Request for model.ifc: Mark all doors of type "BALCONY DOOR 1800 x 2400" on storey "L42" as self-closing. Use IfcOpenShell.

First a look at what the model holds.

```python
import ifcopenshell
import ifcopenshell.util.element

model = ifcopenshell.open("model.ifc")
print(model.schema)
storey = next(s for s in model.by_type("IfcBuildingStorey") if s.Name == "L42")
doors = [e for e in ifcopenshell.util.element.get_decomposition(storey) if e.is_a("IfcDoor")]
seen = {}
for e in doors:
    element_type = ifcopenshell.util.element.get_type(e)
    key = (element_type.Name if element_type != e and element_type else None, ifcopenshell.util.element.get_pset(e, "Pset_DoorCommon", "SelfClosing"))
    seen[key] = seen.get(key, 0) + 1
for (name, value), count in sorted(seen.items(), key=str):
    print(count, "x", name, "|", value)
```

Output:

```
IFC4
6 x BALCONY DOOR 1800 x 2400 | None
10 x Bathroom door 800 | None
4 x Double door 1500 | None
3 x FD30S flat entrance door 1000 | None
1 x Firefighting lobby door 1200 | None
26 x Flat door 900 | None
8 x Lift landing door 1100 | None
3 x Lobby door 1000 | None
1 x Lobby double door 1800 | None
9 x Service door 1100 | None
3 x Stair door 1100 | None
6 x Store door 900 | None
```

```python
import ifcopenshell
import ifcopenshell.api.pset
import ifcopenshell.util.element

model = ifcopenshell.open("model.ifc")

storey = next(s for s in model.by_type("IfcBuildingStorey") if s.Name == "L42")
doors = [e for e in ifcopenshell.util.element.get_decomposition(storey) if e.is_a("IfcDoor")]

count = 0
for e in doors:
    element_type = ifcopenshell.util.element.get_type(e)
    if element_type in (None, e) or element_type.Name != "BALCONY DOOR 1800 x 2400":
        continue
    found = ifcopenshell.util.element.get_pset(e, "Pset_DoorCommon", should_inherit=False)
    if found:
        pset = model.by_id(found["id"])
        if len(ifcopenshell.util.element.get_elements_by_pset(pset)) > 1:
            pset = ifcopenshell.api.pset.unshare_pset(model, products=[e], pset=pset)[0]
    else:
        pset = ifcopenshell.api.pset.add_pset(model, product=e, name="Pset_DoorCommon")
    ifcopenshell.api.pset.edit_pset(model, pset=pset, properties={"SelfClosing": True})
    count += 1

print(count, "doors updated")

model.write("model-out.ifc")
```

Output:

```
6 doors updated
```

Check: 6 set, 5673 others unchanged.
